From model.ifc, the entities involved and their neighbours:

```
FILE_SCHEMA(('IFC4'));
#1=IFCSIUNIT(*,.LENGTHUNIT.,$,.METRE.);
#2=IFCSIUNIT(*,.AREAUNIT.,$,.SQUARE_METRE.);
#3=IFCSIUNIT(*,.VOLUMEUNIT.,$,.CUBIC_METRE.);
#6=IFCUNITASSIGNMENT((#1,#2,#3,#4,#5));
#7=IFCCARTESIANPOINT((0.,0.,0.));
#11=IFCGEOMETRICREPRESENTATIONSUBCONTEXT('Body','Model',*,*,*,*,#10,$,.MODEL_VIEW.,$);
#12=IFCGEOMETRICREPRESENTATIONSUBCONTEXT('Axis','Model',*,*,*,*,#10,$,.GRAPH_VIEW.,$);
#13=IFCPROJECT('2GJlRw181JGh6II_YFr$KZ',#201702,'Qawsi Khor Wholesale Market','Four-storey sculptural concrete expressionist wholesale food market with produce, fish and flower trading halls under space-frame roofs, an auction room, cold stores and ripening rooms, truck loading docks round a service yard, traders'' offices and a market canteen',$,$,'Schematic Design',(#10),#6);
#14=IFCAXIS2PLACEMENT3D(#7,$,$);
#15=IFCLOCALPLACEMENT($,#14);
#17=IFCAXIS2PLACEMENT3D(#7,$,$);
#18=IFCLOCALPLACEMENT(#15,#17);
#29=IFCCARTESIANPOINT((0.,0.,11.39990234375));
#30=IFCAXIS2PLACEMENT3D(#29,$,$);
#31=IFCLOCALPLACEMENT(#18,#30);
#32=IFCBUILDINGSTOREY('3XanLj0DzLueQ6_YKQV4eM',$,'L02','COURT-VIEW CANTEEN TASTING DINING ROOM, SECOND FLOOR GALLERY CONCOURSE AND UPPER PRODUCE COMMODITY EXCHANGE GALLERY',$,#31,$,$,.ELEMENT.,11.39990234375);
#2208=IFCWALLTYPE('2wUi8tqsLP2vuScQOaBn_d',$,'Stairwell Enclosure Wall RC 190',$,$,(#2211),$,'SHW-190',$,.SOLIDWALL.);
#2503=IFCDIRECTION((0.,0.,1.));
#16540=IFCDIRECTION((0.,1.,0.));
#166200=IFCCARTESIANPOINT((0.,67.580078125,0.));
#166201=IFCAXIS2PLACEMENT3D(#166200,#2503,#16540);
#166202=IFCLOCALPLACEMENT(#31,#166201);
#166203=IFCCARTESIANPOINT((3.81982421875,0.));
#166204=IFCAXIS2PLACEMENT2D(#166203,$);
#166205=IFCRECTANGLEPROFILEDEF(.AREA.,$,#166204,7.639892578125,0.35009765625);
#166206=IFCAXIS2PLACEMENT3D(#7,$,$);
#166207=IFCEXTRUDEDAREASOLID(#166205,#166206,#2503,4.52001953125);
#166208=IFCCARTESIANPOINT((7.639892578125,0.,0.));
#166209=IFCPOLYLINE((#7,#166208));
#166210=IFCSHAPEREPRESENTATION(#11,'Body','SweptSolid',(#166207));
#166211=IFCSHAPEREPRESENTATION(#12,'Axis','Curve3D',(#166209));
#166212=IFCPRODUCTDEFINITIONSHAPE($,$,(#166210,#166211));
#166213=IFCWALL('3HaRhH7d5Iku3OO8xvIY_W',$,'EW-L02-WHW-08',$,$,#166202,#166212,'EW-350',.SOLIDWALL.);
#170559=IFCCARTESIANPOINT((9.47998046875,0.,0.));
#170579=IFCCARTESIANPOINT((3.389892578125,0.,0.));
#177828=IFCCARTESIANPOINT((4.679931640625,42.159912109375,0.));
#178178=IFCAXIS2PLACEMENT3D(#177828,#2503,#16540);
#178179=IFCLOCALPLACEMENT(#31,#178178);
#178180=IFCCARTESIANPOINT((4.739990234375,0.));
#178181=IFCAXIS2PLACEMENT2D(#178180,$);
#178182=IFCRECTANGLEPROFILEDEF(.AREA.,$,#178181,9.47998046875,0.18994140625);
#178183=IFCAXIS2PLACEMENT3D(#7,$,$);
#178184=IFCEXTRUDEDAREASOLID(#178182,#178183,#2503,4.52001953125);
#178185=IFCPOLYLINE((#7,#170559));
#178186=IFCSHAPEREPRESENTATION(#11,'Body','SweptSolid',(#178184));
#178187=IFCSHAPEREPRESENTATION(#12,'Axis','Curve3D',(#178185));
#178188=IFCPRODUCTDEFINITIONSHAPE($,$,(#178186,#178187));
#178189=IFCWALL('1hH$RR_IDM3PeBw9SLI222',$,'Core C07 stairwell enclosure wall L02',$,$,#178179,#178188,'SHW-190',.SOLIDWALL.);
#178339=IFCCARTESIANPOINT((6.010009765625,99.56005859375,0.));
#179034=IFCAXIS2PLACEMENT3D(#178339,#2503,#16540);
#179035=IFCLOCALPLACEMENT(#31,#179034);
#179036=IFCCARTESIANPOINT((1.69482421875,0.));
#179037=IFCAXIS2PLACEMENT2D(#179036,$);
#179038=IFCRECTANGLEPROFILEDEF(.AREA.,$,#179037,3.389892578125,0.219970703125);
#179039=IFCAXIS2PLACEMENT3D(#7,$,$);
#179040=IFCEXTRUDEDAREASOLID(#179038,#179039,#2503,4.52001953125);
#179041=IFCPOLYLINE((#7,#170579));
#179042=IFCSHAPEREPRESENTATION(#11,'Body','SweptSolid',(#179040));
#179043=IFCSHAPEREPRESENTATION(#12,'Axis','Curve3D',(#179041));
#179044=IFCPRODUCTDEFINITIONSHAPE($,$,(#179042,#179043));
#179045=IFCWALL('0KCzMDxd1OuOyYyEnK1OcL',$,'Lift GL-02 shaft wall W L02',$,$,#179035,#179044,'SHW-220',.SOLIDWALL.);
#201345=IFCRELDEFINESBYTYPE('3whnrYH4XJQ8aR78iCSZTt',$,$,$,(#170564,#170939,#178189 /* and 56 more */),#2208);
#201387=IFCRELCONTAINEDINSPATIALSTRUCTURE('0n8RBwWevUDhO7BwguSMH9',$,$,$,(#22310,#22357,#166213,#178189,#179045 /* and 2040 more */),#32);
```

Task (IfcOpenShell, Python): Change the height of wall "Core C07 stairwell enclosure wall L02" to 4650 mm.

```python
import ifcopenshell
import ifcopenshell.geom
import ifcopenshell.util.representation
import ifcopenshell.util.shape

model = ifcopenshell.open("model.ifc")
settings = ifcopenshell.geom.settings()


def volume(element):
    """Net volume in cubic metres, openings subtracted."""
    shape = ifcopenshell.geom.create_shape(settings, element)
    return ifcopenshell.util.shape.get_volume(shape.geometry)


wall = model.by_guid("1hH$RR_IDM3PeBw9SLI222")
before = volume(wall)

body = ifcopenshell.util.representation.get_representation(wall, "Model", "Body")
solid = body.Items[0]
old_height = solid.Depth
solid.Depth = 4.65
after = volume(wall)

print(f"height {old_height:g} -> {solid.Depth:g}, volume {before:.3f} -> {after:.3f} m3")

model.write("model_edited.ifc")
```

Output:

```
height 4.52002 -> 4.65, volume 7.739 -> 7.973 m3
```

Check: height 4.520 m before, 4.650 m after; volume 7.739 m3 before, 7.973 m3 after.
